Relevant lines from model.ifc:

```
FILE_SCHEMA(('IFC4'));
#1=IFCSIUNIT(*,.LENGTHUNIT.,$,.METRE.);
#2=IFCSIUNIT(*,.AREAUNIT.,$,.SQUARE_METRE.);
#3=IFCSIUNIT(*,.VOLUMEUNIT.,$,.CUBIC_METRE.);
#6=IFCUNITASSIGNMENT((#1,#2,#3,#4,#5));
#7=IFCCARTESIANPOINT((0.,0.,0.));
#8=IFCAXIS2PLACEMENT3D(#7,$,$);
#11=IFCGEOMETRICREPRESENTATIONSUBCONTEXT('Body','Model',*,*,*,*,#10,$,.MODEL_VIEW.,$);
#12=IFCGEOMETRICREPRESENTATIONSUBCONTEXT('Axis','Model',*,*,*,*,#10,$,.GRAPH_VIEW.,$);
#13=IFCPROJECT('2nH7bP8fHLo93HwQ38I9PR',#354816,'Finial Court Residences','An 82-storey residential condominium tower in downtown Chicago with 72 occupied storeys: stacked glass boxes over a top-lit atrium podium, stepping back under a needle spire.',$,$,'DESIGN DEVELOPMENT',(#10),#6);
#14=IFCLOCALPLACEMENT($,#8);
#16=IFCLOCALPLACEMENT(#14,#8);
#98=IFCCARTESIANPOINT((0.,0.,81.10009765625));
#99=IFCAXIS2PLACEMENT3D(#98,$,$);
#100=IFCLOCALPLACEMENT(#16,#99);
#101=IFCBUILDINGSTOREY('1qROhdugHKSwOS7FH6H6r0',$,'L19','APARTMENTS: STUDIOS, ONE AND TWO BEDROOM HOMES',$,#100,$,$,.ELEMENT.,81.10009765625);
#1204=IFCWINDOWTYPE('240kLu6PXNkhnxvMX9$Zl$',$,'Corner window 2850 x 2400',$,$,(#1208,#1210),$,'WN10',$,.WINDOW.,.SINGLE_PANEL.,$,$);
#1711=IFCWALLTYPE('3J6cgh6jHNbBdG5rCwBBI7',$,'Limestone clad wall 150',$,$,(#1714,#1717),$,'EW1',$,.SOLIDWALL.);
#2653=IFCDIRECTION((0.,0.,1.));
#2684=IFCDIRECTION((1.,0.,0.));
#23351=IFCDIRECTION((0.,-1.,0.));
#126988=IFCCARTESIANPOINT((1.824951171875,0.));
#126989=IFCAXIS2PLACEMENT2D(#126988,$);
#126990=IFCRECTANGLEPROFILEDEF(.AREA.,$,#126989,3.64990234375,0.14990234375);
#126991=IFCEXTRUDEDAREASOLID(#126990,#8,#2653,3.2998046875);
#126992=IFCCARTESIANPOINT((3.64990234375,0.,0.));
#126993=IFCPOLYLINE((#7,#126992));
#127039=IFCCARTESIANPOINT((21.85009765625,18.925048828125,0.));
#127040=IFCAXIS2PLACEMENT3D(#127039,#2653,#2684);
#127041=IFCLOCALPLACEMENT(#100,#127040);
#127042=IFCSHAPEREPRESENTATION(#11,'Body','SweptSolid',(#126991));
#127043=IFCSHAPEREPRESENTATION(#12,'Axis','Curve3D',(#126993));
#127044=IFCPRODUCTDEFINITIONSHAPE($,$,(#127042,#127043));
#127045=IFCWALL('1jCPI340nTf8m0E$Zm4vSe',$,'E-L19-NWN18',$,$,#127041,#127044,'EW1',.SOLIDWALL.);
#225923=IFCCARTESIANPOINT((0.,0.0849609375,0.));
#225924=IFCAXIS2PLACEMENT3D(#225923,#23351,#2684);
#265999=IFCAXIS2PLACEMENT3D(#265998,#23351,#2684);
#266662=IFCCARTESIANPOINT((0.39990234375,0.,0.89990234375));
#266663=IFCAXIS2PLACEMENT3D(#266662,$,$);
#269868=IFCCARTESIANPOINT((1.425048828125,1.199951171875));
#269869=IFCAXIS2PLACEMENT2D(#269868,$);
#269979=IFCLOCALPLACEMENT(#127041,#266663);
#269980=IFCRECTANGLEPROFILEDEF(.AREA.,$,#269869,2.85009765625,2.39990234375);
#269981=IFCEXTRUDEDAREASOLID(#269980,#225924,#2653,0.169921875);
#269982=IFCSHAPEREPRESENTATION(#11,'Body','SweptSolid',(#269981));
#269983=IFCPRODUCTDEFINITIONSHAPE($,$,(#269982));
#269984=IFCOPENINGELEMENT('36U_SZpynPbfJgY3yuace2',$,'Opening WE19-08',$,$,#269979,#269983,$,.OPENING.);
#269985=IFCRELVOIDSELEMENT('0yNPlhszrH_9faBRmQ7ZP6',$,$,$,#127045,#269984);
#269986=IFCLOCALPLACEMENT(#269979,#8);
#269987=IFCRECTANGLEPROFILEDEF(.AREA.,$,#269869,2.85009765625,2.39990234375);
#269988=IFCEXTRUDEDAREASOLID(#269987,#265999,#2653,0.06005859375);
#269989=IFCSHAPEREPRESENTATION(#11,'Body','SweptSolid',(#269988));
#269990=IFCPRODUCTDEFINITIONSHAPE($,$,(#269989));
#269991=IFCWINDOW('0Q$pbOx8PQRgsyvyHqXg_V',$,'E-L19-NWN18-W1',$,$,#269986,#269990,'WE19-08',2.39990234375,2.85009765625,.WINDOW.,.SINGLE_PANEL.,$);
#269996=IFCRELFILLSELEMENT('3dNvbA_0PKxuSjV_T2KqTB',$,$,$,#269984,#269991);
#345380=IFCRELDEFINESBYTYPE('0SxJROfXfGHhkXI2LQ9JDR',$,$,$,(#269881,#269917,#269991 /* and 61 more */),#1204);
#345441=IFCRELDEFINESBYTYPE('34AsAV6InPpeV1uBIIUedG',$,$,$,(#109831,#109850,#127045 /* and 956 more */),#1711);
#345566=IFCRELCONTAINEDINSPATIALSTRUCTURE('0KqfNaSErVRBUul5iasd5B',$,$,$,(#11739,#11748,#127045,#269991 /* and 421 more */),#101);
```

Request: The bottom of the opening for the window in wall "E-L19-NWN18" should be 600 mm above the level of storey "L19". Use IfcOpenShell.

```python
import numpy as np
import ifcopenshell
import ifcopenshell.api.geometry
import ifcopenshell.geom
import ifcopenshell.util.element
import ifcopenshell.util.placement
import ifcopenshell.util.shape
import ifcopenshell.util.unit

model = ifcopenshell.open("model.ifc")
unit_scale = ifcopenshell.util.unit.calculate_unit_scale(model)

window = model.by_guid("0Q$pbOx8PQRgsyvyHqXg_V")
opening = window.FillsVoids[0].RelatingOpeningElement
storey = ifcopenshell.util.element.get_container(window, ifc_class="IfcBuildingStorey")
level = ifcopenshell.util.placement.get_local_placement(storey.ObjectPlacement)[2, 3]

# The opening's origin need not be at the sill, so measure its lowest point.
shape = ifcopenshell.geom.create_shape(ifcopenshell.geom.settings(), opening)
bottom = ifcopenshell.util.shape.get_shape_bottom_elevation(shape, shape.geometry) / unit_scale
dz = level + 0.6 / unit_scale - bottom

shift = np.array([0.0, 0.0, dz])
# The window is placed relative to its opening, so it follows when the opening moves.
matrix = ifcopenshell.util.placement.get_local_placement(opening.ObjectPlacement)
matrix[:3, 3] += shift
ifcopenshell.api.geometry.edit_object_placement(
    model, product=opening, matrix=matrix, is_si=False, should_transform_children=True
)

print(f"moved by {dz * unit_scale:+.3f} m")

model.write("model_v2.ifc")
```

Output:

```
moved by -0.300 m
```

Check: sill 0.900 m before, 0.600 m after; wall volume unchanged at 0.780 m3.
